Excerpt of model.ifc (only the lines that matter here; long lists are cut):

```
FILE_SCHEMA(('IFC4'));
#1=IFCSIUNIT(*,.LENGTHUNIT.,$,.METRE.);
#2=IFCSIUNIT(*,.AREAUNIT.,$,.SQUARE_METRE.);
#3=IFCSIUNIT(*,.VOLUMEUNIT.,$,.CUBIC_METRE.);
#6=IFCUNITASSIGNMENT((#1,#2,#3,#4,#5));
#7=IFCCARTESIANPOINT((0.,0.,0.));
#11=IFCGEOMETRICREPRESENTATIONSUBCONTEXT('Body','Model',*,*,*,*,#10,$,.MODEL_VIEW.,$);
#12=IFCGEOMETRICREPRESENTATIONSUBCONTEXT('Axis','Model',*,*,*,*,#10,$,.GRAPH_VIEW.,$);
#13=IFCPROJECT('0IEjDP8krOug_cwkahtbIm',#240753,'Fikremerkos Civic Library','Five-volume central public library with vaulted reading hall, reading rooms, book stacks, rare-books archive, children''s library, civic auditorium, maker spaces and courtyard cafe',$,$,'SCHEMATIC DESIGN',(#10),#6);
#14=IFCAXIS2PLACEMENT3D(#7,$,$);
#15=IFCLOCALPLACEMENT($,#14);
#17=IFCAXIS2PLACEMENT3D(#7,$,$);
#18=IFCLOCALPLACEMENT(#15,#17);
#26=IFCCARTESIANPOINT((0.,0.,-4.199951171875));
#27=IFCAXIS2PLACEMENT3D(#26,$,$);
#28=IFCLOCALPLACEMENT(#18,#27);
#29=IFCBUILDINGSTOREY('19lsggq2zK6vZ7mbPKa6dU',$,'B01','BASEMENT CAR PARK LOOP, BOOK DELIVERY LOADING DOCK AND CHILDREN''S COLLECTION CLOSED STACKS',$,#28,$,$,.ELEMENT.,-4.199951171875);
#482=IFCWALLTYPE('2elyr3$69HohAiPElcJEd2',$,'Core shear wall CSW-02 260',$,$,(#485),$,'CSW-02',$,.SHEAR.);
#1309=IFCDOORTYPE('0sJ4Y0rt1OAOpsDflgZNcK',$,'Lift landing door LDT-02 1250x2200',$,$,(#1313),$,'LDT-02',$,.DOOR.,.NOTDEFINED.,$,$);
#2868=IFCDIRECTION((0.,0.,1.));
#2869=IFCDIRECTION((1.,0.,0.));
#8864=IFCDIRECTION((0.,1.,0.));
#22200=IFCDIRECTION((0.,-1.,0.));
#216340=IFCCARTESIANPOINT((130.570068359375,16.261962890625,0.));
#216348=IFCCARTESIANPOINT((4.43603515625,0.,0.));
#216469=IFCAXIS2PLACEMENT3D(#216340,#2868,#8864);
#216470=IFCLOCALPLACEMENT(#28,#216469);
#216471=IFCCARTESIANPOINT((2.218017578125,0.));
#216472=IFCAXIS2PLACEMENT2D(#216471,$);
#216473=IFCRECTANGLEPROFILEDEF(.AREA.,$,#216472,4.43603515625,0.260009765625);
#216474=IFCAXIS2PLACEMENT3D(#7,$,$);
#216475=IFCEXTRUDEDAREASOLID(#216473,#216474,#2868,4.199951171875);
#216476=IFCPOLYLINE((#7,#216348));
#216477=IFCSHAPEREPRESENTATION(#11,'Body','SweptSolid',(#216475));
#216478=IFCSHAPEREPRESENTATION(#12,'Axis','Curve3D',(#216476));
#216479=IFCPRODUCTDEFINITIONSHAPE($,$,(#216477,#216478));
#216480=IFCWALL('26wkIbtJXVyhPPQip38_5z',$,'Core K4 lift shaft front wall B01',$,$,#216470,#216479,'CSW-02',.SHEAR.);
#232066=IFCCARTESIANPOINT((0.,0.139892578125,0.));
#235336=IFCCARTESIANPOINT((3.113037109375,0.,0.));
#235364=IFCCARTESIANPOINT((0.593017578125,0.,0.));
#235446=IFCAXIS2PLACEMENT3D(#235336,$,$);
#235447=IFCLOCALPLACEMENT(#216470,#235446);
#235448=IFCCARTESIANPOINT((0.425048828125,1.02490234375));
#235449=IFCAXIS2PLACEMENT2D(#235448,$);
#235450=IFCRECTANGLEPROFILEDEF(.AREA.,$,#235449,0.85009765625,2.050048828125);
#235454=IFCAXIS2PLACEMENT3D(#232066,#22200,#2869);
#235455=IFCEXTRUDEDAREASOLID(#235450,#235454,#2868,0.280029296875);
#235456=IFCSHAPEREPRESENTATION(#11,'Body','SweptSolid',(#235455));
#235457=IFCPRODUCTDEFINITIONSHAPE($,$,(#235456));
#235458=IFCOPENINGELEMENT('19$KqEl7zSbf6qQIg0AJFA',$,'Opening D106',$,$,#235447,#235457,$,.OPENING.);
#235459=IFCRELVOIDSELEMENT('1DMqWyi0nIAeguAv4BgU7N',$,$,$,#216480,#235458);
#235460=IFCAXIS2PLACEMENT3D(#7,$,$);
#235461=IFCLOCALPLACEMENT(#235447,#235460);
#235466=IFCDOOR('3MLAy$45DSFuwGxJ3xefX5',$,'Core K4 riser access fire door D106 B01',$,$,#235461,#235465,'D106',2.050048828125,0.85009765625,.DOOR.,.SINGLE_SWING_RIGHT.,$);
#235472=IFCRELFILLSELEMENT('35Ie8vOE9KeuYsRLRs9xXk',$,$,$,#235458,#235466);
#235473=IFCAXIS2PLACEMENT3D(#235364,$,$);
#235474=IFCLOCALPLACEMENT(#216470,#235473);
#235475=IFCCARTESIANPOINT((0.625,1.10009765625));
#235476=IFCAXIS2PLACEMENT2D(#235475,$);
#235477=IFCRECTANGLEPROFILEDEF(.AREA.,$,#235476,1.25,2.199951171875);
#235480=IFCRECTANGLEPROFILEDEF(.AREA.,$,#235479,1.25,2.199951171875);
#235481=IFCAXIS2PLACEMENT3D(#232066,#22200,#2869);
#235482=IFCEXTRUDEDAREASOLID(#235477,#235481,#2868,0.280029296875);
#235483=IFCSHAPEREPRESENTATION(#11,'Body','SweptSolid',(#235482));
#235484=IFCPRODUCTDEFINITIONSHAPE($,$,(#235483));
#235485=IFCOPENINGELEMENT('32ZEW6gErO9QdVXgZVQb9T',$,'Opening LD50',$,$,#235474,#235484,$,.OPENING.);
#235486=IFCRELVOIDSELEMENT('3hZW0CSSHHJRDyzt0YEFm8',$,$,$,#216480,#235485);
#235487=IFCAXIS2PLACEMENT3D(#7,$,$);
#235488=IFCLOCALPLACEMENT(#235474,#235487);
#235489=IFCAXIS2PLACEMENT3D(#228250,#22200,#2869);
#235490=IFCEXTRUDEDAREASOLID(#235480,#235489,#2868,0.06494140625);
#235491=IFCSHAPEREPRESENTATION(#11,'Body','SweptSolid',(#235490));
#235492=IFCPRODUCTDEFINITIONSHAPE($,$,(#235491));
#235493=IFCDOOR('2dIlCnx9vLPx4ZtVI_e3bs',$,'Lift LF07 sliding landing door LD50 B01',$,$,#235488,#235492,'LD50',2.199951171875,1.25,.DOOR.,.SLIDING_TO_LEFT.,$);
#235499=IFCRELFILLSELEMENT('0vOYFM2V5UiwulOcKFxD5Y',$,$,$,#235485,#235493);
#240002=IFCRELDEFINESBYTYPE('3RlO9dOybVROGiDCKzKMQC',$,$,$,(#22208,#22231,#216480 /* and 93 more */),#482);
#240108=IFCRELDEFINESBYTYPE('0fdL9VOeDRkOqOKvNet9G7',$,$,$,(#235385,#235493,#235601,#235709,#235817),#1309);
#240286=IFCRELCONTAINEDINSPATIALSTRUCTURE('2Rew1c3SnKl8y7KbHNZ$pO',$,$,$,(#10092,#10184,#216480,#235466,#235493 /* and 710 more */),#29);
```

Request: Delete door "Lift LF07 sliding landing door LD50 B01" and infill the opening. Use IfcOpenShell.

```python
import ifcopenshell
import ifcopenshell.api.feature
import ifcopenshell.api.root
import ifcopenshell.geom
import ifcopenshell.util.shape

model = ifcopenshell.open("model.ifc")
settings = ifcopenshell.geom.settings()


def volume(element):
    """Net volume in cubic metres, openings subtracted."""
    shape = ifcopenshell.geom.create_shape(settings, element)
    return ifcopenshell.util.shape.get_volume(shape.geometry)


door = model.by_guid("2dIlCnx9vLPx4ZtVI_e3bs")
opening = door.FillsVoids[0].RelatingOpeningElement
wall = opening.VoidsElements[0].RelatingBuildingElement
before = volume(wall)

ifcopenshell.api.root.remove_product(model, product=door)
ifcopenshell.api.feature.remove_feature(model, feature=opening)

after = volume(wall)

print(f"wall volume {before:.3f} -> {after:.3f} m3")

model.write("model_v2.ifc")
```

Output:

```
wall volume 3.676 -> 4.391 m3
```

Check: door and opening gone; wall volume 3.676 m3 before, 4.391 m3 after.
